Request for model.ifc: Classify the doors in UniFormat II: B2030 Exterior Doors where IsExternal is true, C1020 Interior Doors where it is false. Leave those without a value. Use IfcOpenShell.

First a look at what the model holds.

```python
import ifcopenshell
import ifcopenshell.util.element

model = ifcopenshell.open("model.ifc")
print(model.schema)
print("classifications:", [c.Name for c in model.by_type("IfcClassification")])
values = [ifcopenshell.util.element.get_pset(e, "Pset_DoorCommon", "IsExternal") for e in model.by_type("IfcDoor")]
for value in (True, False, None):
    print("IsExternal", value, values.count(value))
```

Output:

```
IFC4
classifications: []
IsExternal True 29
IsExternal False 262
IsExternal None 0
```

```python
import ifcopenshell
import ifcopenshell.api.classification
import ifcopenshell.util.element

model = ifcopenshell.open("model.ifc")

system = ifcopenshell.api.classification.add_classification(model, classification="UniFormat II")

doors = model.by_type("IfcDoor")
external = {e: ifcopenshell.util.element.get_pset(e, "Pset_DoorCommon", "IsExternal") for e in doors}
for flag, code, name in ((True, "B2030", "Exterior Doors"), (False, "C1020", "Interior Doors")):
    products = [e for e in doors if external[e] is flag]
    ifcopenshell.api.classification.add_reference(
        model, products=products, classification=system, identification=code, name=name
    )
    print(code, len(products))

model.write("model_v2.ifc")
```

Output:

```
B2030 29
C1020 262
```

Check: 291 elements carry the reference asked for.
